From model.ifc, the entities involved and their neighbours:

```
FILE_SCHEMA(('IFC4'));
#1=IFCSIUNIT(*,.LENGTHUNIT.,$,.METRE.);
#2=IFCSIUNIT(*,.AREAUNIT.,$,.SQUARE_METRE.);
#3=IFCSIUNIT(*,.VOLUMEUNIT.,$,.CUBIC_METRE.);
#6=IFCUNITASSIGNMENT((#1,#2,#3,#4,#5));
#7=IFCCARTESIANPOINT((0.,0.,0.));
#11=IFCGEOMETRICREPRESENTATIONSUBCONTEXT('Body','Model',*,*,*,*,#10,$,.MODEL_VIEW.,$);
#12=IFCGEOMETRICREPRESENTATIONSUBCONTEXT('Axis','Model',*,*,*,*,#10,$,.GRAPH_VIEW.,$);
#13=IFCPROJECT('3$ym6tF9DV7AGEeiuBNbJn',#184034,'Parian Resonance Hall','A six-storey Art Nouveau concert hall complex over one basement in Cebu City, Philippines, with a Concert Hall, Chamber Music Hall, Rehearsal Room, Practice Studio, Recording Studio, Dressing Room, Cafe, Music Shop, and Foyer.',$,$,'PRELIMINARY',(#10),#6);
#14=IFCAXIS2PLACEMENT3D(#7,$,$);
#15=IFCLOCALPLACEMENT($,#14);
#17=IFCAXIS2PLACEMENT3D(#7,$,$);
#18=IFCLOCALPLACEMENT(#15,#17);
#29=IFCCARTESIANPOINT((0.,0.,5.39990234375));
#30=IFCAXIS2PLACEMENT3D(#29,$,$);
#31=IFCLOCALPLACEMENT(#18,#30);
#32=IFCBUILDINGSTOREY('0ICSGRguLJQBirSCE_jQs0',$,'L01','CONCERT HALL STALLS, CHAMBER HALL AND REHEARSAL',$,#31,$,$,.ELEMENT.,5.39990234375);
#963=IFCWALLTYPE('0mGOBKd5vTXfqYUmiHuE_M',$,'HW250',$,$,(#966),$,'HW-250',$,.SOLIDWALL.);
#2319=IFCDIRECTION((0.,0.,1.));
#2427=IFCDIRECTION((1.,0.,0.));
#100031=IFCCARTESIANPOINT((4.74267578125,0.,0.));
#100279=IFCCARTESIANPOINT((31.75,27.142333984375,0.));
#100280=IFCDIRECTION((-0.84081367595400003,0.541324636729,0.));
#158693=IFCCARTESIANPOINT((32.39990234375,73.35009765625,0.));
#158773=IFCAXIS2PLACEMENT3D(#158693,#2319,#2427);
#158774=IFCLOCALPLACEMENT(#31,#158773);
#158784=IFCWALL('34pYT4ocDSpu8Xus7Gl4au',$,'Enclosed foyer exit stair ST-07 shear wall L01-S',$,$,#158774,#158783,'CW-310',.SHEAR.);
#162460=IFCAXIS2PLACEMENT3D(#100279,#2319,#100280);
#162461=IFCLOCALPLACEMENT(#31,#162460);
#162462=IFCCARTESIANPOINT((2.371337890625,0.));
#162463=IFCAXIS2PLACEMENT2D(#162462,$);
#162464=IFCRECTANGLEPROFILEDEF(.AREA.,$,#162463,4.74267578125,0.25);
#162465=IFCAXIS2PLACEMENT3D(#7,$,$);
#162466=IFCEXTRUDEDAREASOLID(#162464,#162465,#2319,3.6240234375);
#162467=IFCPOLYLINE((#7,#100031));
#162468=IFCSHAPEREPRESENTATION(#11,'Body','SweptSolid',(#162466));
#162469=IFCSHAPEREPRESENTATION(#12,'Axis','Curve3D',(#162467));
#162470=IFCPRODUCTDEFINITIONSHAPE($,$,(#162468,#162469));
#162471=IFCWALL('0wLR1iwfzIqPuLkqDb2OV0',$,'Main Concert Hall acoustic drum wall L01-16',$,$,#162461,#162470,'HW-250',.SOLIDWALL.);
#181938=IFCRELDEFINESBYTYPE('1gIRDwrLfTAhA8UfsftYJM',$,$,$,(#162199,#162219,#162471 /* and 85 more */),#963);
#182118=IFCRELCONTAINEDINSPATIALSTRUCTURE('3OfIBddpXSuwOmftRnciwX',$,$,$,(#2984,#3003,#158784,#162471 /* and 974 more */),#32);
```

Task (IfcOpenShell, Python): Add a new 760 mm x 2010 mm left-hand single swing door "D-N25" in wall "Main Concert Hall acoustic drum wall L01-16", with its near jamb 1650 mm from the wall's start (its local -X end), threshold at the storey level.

```python
import numpy as np
import ifcopenshell
import ifcopenshell.api.feature
import ifcopenshell.api.geometry
import ifcopenshell.api.root
import ifcopenshell.api.spatial
import ifcopenshell.geom
import ifcopenshell.util.element
import ifcopenshell.util.placement
import ifcopenshell.util.representation
import ifcopenshell.util.shape
import ifcopenshell.util.unit

model = ifcopenshell.open("model.ifc")
unit_scale = ifcopenshell.util.unit.calculate_unit_scale(model)
settings = ifcopenshell.geom.settings()


def volume(element):
    """Net volume in cubic metres, openings subtracted."""
    shape = ifcopenshell.geom.create_shape(settings, element)
    return ifcopenshell.util.shape.get_volume(shape.geometry)


wall = model.by_guid("0wLR1iwfzIqPuLkqDb2OV0")
storey = ifcopenshell.util.element.get_container(wall, ifc_class="IfcBuildingStorey")
context = ifcopenshell.util.representation.get_context(model, "Model", "Body", "MODEL_VIEW")
before = volume(wall)

width, height, from_end, sill = 0.76, 2.01, 1.65, 0.0  # metres

# The wall runs along its own X axis, and the end named is its -X end.
wall_shape = ifcopenshell.geom.create_shape(settings, wall)
x, y, z = ifcopenshell.util.shape.get_vertices(wall_shape.geometry).T
start = x.min() + from_end
face, thickness = float(y.min()), float(y.max() - y.min())
wall_matrix = ifcopenshell.util.placement.get_local_placement(wall.ObjectPlacement)
level = ifcopenshell.util.placement.get_local_placement(storey.ObjectPlacement)[2, 3]


def in_wall(x, y):
    """Placement at x, y metres in the wall's axes, at sill height."""
    matrix = wall_matrix.copy()
    matrix[:, 3] = wall_matrix @ np.array([x / unit_scale, y / unit_scale, 0.0, 1.0])
    matrix[2, 3] = level + sill / unit_scale
    return matrix


# Opening: a box that overshoots both wall faces by 50 mm.
opening = ifcopenshell.api.root.create_entity(model, ifc_class="IfcOpeningElement", predefined_type="OPENING")
box = ifcopenshell.api.geometry.add_wall_representation(
    model, context=context, length=width, height=height, thickness=thickness + 0.1
)
ifcopenshell.api.geometry.assign_representation(model, product=opening, representation=box)
ifcopenshell.api.geometry.edit_object_placement(model, product=opening, matrix=in_wall(start, face - 0.05), is_si=False)
ifcopenshell.api.feature.add_feature(model, feature=opening, element=wall)

door = ifcopenshell.api.root.create_entity(model, ifc_class="IfcDoor", name="D-N25", predefined_type="DOOR")
door.OverallWidth, door.OverallHeight = width / unit_scale, height / unit_scale
door.OperationType = "SINGLE_SWING_LEFT"
body = ifcopenshell.api.geometry.add_door_representation(
    model,
    context=context,
    overall_width=door.OverallWidth,
    overall_height=door.OverallHeight,
    operation_type="SINGLE_SWING_LEFT",
    lining_properties={"LiningDepth": thickness / unit_scale, "ThresholdDepth": thickness / unit_scale},
)
ifcopenshell.api.geometry.assign_representation(model, product=door, representation=body)
ifcopenshell.api.spatial.assign_container(model, products=[door], relating_structure=storey)
ifcopenshell.api.feature.add_filling(model, opening=opening, element=door)

# The lining spans the wall, so the door starts at the wall face.
ifcopenshell.api.geometry.edit_object_placement(model, product=door, matrix=in_wall(start, face), is_si=False)

after = volume(wall)

print(f"wall volume {before:.3f} -> {after:.3f} m3")

model.write("model_v2.ifc")
```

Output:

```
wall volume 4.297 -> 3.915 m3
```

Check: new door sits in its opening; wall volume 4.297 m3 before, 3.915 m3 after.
